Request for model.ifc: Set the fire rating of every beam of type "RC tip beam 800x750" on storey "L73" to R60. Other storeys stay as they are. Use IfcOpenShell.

First a look at what the model holds.

```python
import ifcopenshell
import ifcopenshell.util.element

model = ifcopenshell.open("model.ifc")
print(model.schema)
storey = next(s for s in model.by_type("IfcBuildingStorey") if s.Name == "L73")
beams = [e for e in ifcopenshell.util.element.get_decomposition(storey) if e.is_a("IfcBeam")]
seen = {}
for e in beams:
    element_type = ifcopenshell.util.element.get_type(e)
    key = (element_type.Name if element_type != e and element_type else None, ifcopenshell.util.element.get_pset(e, "Pset_BeamCommon", "FireRating"))
    seen[key] = seen.get(key, 0) + 1
for (name, value), count in sorted(seen.items(), key=str):
    print(count, "x", name, "|", value)
```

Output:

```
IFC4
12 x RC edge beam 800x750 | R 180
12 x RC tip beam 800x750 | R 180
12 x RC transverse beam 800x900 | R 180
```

```python
import ifcopenshell
import ifcopenshell.api.pset
import ifcopenshell.util.element

model = ifcopenshell.open("model.ifc")

storey = next(s for s in model.by_type("IfcBuildingStorey") if s.Name == "L73")
beams = [e for e in ifcopenshell.util.element.get_decomposition(storey) if e.is_a("IfcBeam")]

count = 0
for e in beams:
    element_type = ifcopenshell.util.element.get_type(e)
    if element_type in (None, e) or element_type.Name != "RC tip beam 800x750":
        continue
    found = ifcopenshell.util.element.get_pset(e, "Pset_BeamCommon", should_inherit=False)
    if found:
        pset = model.by_id(found["id"])
        if len(ifcopenshell.util.element.get_elements_by_pset(pset)) > 1:
            pset = ifcopenshell.api.pset.unshare_pset(model, products=[e], pset=pset)[0]
    else:
        pset = ifcopenshell.api.pset.add_pset(model, product=e, name="Pset_BeamCommon")
    ifcopenshell.api.pset.edit_pset(model, pset=pset, properties={"FireRating": "R60"})
    count += 1

print(count, "beams updated")

model.write("model-out.ifc")
```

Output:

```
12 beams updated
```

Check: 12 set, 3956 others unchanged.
